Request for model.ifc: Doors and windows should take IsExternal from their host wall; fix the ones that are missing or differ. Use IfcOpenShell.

First a look at what the model holds.

```python
import ifcopenshell
import ifcopenshell.util.element

model = ifcopenshell.open("model.ifc")
print(model.schema)
seen = {}
for e in model.by_type("IfcDoor") + model.by_type("IfcWindow"):
    if not e.FillsVoids:
        continue
    host = e.FillsVoids[0].RelatingOpeningElement.VoidsElements[0].RelatingBuildingElement
    own = ifcopenshell.util.element.get_pset(e, f"Pset_{e.is_a()[3:].removesuffix('StandardCase')}Common", "IsExternal")
    wall = ifcopenshell.util.element.get_pset(host, "Pset_WallCommon", "IsExternal")
    seen[e.is_a(), own, wall] = seen.get((e.is_a(), own, wall), 0) + 1
for (cls, own, wall), count in sorted(seen.items(), key=str):
    print(count, cls, "IsExternal:", own, "| host wall:", wall)
```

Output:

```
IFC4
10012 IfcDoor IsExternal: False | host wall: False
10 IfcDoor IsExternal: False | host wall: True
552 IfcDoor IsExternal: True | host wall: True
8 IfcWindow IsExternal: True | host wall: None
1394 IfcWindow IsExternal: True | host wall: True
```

```python
import ifcopenshell
import ifcopenshell.api.pset
import ifcopenshell.util.element

model = ifcopenshell.open("model.ifc")

count = 0
for ifc_class, pset_name in (("IfcDoor", "Pset_DoorCommon"), ("IfcWindow", "Pset_WindowCommon")):
    for e in model.by_type(ifc_class):
        if not e.FillsVoids:
            continue
        host = e.FillsVoids[0].RelatingOpeningElement.VoidsElements[0].RelatingBuildingElement
        external = ifcopenshell.util.element.get_pset(host, "Pset_WallCommon", "IsExternal")
        if external is None or ifcopenshell.util.element.get_pset(e, pset_name, "IsExternal") == external:
            continue
        found = ifcopenshell.util.element.get_pset(e, pset_name, should_inherit=False)
        if found:
            pset = model.by_id(found["id"])
            if len(ifcopenshell.util.element.get_elements_by_pset(pset)) > 1:
                pset = ifcopenshell.api.pset.unshare_pset(model, products=[e], pset=pset)[0]
        else:
            pset = ifcopenshell.api.pset.add_pset(model, product=e, name=pset_name)
        ifcopenshell.api.pset.edit_pset(model, pset=pset, properties={"IsExternal": external})
        count += 1

print(count, "updated")

model.write("model_updated.ifc")
```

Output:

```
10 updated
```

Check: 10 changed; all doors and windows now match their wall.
